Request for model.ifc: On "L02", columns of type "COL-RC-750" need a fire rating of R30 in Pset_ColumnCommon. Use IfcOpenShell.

First a look at what the model holds.

```python
import ifcopenshell
import ifcopenshell.util.element

model = ifcopenshell.open("model.ifc")
print(model.schema)
storey = next(s for s in model.by_type("IfcBuildingStorey") if s.Name == "L02")
columns = [e for e in ifcopenshell.util.element.get_decomposition(storey) if e.is_a("IfcColumn")]
seen = {}
for e in columns:
    element_type = ifcopenshell.util.element.get_type(e)
    key = (element_type.Name if element_type != e and element_type else None, ifcopenshell.util.element.get_pset(e, "Pset_ColumnCommon", "FireRating"))
    seen[key] = seen.get(key, 0) + 1
for (name, value), count in sorted(seen.items(), key=str):
    print(count, "x", name, "|", value)
```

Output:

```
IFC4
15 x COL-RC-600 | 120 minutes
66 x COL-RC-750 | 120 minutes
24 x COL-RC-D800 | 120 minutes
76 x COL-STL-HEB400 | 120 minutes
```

```python
import ifcopenshell
import ifcopenshell.api.pset
import ifcopenshell.util.element

model = ifcopenshell.open("model.ifc")

storey = next(s for s in model.by_type("IfcBuildingStorey") if s.Name == "L02")
columns = [e for e in ifcopenshell.util.element.get_decomposition(storey) if e.is_a("IfcColumn")]

count = 0
for e in columns:
    element_type = ifcopenshell.util.element.get_type(e)
    if element_type in (None, e) or element_type.Name != "COL-RC-750":
        continue
    # add_pset returns the element's existing set when there is one.
    pset = ifcopenshell.api.pset.add_pset(model, product=e, name="Pset_ColumnCommon")
    ifcopenshell.api.pset.edit_pset(model, pset=pset, properties={"FireRating": "R30"})
    count += 1

print(count, "columns updated")

model.write("model_rev.ifc")
```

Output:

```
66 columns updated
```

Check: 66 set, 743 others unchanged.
